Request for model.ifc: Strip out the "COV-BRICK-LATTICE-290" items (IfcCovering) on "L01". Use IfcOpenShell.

First a look at what the model holds.

```python
import ifcopenshell
import ifcopenshell.util.element

model = ifcopenshell.open("model.ifc")
print(model.schema)
storey = next(s for s in model.by_type("IfcBuildingStorey") if s.Name == "L01")
coverings = [e for e in ifcopenshell.util.element.get_decomposition(storey) if e.is_a("IfcCovering")]
seen = {}
for e in coverings:
    element_type = ifcopenshell.util.element.get_type(e)
    name = element_type.Name if element_type not in (None, e) else None
    seen[name] = seen.get(name, 0) + 1
for name, count in sorted(seen.items(), key=str):
    print(count, "x", name)
```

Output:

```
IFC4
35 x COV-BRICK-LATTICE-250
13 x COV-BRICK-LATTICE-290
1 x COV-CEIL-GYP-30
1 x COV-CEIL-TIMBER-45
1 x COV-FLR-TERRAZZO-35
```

```python
import ifcopenshell
import ifcopenshell.api.root
import ifcopenshell.util.element

model = ifcopenshell.open("model.ifc")

storey = next(s for s in model.by_type("IfcBuildingStorey") if s.Name == "L01")
coverings = [e for e in ifcopenshell.util.element.get_decomposition(storey) if e.is_a("IfcCovering")]
targets = [e for e in coverings if (t := ifcopenshell.util.element.get_type(e)) not in (None, e) and t.Name == "COV-BRICK-LATTICE-290"]

for e in targets:
    ifcopenshell.api.root.remove_product(model, product=e)
print(len(targets), "removed")

model.write("model-out.ifc")
```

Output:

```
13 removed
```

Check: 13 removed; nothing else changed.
